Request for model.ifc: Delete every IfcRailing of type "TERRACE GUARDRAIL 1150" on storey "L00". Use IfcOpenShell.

First a look at what the model holds.

```python
import ifcopenshell
import ifcopenshell.util.element

model = ifcopenshell.open("model.ifc")
print(model.schema)
storey = next(s for s in model.by_type("IfcBuildingStorey") if s.Name == "L00")
railings = [e for e in ifcopenshell.util.element.get_decomposition(storey) if e.is_a("IfcRailing")]
seen = {}
for e in railings:
    element_type = ifcopenshell.util.element.get_type(e)
    name = element_type.Name if element_type not in (None, e) else None
    seen[name] = seen.get(name, 0) + 1
for name, count in sorted(seen.items(), key=str):
    print(count, "x", name)
```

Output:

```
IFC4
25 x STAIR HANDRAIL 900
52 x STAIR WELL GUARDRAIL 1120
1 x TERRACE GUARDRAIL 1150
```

```python
import ifcopenshell
import ifcopenshell.api.root
import ifcopenshell.util.element

model = ifcopenshell.open("model.ifc")

storey = next(s for s in model.by_type("IfcBuildingStorey") if s.Name == "L00")
railings = [e for e in ifcopenshell.util.element.get_decomposition(storey) if e.is_a("IfcRailing")]
targets = [e for e in railings if (t := ifcopenshell.util.element.get_type(e)) not in (None, e) and t.Name == "TERRACE GUARDRAIL 1150"]

for e in targets:
    ifcopenshell.api.root.remove_product(model, product=e)
print(len(targets), "removed")

model.write("model_edited.ifc")
```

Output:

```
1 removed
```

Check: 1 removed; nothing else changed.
